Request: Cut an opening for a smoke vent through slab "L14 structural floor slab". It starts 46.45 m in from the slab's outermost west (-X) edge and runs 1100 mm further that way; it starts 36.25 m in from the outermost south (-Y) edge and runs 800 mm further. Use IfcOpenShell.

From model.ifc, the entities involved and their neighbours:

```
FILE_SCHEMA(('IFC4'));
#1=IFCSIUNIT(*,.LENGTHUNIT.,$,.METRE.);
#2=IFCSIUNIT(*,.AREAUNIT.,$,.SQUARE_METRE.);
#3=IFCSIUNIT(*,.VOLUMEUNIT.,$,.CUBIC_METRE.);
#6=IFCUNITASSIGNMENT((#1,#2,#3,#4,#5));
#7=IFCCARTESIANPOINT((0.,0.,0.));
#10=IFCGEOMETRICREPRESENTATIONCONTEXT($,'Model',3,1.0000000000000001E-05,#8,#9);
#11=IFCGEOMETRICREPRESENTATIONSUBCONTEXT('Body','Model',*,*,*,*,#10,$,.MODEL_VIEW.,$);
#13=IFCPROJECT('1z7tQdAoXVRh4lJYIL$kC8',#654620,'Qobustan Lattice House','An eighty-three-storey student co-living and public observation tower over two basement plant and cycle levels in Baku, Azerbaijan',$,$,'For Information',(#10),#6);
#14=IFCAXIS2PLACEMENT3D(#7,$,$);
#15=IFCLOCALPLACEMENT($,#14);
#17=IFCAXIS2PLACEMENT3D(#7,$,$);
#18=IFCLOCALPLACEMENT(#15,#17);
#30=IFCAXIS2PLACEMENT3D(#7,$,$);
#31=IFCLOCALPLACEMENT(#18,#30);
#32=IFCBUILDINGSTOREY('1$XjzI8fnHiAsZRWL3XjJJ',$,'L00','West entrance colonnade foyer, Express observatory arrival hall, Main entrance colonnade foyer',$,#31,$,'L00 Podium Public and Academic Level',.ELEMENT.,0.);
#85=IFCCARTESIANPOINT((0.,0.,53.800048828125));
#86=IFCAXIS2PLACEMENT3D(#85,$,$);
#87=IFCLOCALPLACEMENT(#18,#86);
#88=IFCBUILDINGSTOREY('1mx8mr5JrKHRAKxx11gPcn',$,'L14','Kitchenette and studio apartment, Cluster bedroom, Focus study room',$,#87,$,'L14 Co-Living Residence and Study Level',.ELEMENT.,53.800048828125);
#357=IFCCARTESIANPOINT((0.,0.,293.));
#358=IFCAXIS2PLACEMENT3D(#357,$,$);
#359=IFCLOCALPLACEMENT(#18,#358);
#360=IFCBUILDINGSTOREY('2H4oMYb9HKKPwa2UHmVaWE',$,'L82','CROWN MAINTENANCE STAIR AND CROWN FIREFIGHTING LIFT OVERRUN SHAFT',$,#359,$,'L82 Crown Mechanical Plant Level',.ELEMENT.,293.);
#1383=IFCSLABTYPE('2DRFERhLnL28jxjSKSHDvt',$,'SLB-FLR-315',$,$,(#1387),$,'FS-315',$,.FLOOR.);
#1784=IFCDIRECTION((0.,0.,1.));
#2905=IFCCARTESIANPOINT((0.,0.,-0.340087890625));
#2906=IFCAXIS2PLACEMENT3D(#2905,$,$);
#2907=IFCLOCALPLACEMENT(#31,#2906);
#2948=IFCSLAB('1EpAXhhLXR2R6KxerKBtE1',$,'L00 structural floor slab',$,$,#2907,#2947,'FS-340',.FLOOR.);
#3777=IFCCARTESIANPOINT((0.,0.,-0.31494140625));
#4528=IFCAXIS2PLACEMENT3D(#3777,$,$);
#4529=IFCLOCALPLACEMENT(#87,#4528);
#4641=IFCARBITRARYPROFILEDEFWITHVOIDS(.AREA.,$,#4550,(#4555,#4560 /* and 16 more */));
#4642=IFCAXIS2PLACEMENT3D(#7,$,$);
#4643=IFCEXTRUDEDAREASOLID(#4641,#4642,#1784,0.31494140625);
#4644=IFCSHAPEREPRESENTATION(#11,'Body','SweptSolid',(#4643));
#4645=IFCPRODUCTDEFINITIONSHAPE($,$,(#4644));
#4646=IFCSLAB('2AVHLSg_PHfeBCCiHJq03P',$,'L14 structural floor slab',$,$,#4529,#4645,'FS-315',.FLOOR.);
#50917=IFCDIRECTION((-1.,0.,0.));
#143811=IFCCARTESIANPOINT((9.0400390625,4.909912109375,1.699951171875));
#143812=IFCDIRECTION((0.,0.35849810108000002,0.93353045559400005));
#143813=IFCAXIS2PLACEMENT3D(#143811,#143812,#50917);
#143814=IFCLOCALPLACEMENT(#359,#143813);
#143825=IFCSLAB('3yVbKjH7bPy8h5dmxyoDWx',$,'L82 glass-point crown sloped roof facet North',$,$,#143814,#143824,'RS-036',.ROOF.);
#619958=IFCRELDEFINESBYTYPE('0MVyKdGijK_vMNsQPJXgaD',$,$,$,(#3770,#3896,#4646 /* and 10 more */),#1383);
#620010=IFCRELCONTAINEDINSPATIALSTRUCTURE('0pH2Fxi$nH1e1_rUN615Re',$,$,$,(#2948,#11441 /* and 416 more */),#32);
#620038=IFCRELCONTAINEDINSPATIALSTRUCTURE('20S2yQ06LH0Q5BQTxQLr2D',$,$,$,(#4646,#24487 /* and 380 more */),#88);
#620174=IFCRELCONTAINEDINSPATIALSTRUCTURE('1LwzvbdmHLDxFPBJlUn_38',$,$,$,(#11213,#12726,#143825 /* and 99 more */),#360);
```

```python
import numpy as np
import ifcopenshell
import ifcopenshell.api.feature
import ifcopenshell.api.geometry
import ifcopenshell.api.root
import ifcopenshell.geom
import ifcopenshell.util.placement
import ifcopenshell.util.representation
import ifcopenshell.util.shape
import ifcopenshell.util.unit

model = ifcopenshell.open("model.ifc")
unit_scale = ifcopenshell.util.unit.calculate_unit_scale(model)
settings = ifcopenshell.geom.settings()


def volume(element):
    """Net volume in cubic metres, openings subtracted."""
    shape = ifcopenshell.geom.create_shape(settings, element)
    return ifcopenshell.util.shape.get_volume(shape.geometry)


slab = model.by_id(4646)
before = volume(slab)

# Extent in the slab's own axes, in metres. The edges named are its -X and -Y sides.
slab_shape = ifcopenshell.geom.create_shape(settings, slab)
vertices = ifcopenshell.util.shape.get_vertices(slab_shape.geometry)
x_min, y_min, bottom = vertices.min(axis=0)
top = vertices[:, 2].max()

opening = ifcopenshell.api.root.create_entity(model, ifc_class="IfcOpeningElement", name="Smoke vent opening", predefined_type="OPENING")
context = ifcopenshell.util.representation.get_context(model, "Model", "Body", "MODEL_VIEW")
width, depth = 1.1, 0.8
outline = [(0.0, 0.0), (width, 0.0), (width, depth), (0.0, depth), (0.0, 0.0)]
# Overshoot both faces by 50 mm so the cut is clean.
shape = ifcopenshell.api.geometry.add_slab_representation(
    model, context=context, depth=top - bottom + 0.1, polyline=outline
)
ifcopenshell.api.geometry.assign_representation(model, product=opening, representation=shape)

matrix = ifcopenshell.util.placement.get_local_placement(slab.ObjectPlacement)
matrix[:, 3] = matrix @ np.append(np.array([x_min + 46.45, y_min + 36.25, bottom - 0.05]) / unit_scale, 1.0)
ifcopenshell.api.geometry.edit_object_placement(model, product=opening, matrix=matrix, is_si=False)
ifcopenshell.api.feature.add_feature(model, feature=opening, element=slab)

after = volume(slab)

print(f"slab volume {before:.3f} -> {after:.3f} m3")

model.write("model-out.ifc")
```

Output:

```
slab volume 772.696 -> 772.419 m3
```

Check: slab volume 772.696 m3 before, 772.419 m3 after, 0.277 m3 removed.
